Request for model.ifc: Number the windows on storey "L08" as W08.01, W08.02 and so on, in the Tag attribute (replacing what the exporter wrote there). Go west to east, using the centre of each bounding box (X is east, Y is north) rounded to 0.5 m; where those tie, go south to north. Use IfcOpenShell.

First a look at what the model holds.

```python
import ifcopenshell
import ifcopenshell.util.element
import ifcopenshell.util.placement

model = ifcopenshell.open("model.ifc")
print(model.schema)
storey = next(s for s in model.by_type("IfcBuildingStorey") if s.Name == "L08")
windows = [e for e in ifcopenshell.util.element.get_decomposition(storey) if e.is_a("IfcWindow")]
for e in sorted(windows, key=lambda e: e.id()):
    origin = ifcopenshell.util.placement.get_local_placement(e.ObjectPlacement)[:3, 3]
    print(e.id(), e.Tag, e.Name, origin.round(2) + 0.0, sep=" | ")
```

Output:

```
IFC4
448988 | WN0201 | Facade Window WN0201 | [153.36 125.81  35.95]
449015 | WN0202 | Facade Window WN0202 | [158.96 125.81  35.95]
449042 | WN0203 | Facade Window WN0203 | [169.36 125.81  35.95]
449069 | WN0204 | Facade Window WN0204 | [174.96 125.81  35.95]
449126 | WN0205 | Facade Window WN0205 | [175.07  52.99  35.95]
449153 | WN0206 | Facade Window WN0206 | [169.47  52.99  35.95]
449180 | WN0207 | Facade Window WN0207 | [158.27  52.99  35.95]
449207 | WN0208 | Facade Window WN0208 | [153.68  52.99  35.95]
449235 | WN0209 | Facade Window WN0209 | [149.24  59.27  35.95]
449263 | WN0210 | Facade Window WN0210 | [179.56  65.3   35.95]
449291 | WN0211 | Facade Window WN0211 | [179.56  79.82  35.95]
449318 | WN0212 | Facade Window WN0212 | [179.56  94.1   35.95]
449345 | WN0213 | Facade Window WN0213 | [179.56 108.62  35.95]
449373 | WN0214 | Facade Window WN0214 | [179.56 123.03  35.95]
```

```python
import ifcopenshell
import ifcopenshell.geom
import ifcopenshell.util.element
import ifcopenshell.util.shape

model = ifcopenshell.open("model.ifc")
settings = ifcopenshell.geom.settings()
settings.set("use-world-coords", True)


def centre(element):
    shape = ifcopenshell.geom.create_shape(settings, element)
    return ifcopenshell.util.shape.get_bbox_centroid(shape.geometry)


storey = next(s for s in model.by_type("IfcBuildingStorey") if s.Name == "L08")
windows = [e for e in ifcopenshell.util.element.get_decomposition(storey) if e.is_a("IfcWindow")]

# Insertion points can sit at a corner or the storey origin, so sort by the geometry (in metres).
centres = {e: centre(e) for e in windows}
windows.sort(key=lambda e: (round(centres[e][0] / 0.5), centres[e][1]))

for i, e in enumerate(windows, start=1):
    number = f"W08.{i:02d}"
    e.Tag = number
    print(e.id(), number)

model.write("model-out.ifc")
```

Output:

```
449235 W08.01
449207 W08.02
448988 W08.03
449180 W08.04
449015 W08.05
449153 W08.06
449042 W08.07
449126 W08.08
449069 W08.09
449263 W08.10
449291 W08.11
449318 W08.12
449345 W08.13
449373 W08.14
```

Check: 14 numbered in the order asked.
